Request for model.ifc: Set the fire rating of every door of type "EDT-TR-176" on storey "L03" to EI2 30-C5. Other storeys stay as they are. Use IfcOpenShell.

First a look at what the model holds.

```python
import ifcopenshell
import ifcopenshell.util.element

model = ifcopenshell.open("model.ifc")
print(model.schema)
storey = next(s for s in model.by_type("IfcBuildingStorey") if s.Name == "L03")
doors = [e for e in ifcopenshell.util.element.get_decomposition(storey) if e.is_a("IfcDoor")]
seen = {}
for e in doors:
    element_type = ifcopenshell.util.element.get_type(e)
    key = (element_type.Name if element_type != e and element_type else None, ifcopenshell.util.element.get_pset(e, "Pset_DoorCommon", "FireRating"))
    seen[key] = seen.get(key, 0) + 1
for (name, value), count in sorted(seen.items(), key=str):
    print(count, "x", name, "|", value)
```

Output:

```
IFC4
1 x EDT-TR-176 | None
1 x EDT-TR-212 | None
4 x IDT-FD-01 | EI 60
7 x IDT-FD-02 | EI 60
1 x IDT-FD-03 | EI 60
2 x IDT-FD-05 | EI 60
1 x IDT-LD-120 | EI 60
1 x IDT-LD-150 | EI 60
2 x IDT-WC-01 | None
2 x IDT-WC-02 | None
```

```python
import ifcopenshell
import ifcopenshell.api.pset
import ifcopenshell.util.element

model = ifcopenshell.open("model.ifc")

storey = next(s for s in model.by_type("IfcBuildingStorey") if s.Name == "L03")
doors = [e for e in ifcopenshell.util.element.get_decomposition(storey) if e.is_a("IfcDoor")]

count = 0
for e in doors:
    element_type = ifcopenshell.util.element.get_type(e)
    if element_type in (None, e) or element_type.Name != "EDT-TR-176":
        continue
    # add_pset returns the element's existing set when there is one.
    pset = ifcopenshell.api.pset.add_pset(model, product=e, name="Pset_DoorCommon")
    ifcopenshell.api.pset.edit_pset(model, pset=pset, properties={"FireRating": "EI2 30-C5"})
    count += 1

print(count, "doors updated")

model.write("model_updated.ifc")
```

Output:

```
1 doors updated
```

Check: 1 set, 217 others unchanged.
